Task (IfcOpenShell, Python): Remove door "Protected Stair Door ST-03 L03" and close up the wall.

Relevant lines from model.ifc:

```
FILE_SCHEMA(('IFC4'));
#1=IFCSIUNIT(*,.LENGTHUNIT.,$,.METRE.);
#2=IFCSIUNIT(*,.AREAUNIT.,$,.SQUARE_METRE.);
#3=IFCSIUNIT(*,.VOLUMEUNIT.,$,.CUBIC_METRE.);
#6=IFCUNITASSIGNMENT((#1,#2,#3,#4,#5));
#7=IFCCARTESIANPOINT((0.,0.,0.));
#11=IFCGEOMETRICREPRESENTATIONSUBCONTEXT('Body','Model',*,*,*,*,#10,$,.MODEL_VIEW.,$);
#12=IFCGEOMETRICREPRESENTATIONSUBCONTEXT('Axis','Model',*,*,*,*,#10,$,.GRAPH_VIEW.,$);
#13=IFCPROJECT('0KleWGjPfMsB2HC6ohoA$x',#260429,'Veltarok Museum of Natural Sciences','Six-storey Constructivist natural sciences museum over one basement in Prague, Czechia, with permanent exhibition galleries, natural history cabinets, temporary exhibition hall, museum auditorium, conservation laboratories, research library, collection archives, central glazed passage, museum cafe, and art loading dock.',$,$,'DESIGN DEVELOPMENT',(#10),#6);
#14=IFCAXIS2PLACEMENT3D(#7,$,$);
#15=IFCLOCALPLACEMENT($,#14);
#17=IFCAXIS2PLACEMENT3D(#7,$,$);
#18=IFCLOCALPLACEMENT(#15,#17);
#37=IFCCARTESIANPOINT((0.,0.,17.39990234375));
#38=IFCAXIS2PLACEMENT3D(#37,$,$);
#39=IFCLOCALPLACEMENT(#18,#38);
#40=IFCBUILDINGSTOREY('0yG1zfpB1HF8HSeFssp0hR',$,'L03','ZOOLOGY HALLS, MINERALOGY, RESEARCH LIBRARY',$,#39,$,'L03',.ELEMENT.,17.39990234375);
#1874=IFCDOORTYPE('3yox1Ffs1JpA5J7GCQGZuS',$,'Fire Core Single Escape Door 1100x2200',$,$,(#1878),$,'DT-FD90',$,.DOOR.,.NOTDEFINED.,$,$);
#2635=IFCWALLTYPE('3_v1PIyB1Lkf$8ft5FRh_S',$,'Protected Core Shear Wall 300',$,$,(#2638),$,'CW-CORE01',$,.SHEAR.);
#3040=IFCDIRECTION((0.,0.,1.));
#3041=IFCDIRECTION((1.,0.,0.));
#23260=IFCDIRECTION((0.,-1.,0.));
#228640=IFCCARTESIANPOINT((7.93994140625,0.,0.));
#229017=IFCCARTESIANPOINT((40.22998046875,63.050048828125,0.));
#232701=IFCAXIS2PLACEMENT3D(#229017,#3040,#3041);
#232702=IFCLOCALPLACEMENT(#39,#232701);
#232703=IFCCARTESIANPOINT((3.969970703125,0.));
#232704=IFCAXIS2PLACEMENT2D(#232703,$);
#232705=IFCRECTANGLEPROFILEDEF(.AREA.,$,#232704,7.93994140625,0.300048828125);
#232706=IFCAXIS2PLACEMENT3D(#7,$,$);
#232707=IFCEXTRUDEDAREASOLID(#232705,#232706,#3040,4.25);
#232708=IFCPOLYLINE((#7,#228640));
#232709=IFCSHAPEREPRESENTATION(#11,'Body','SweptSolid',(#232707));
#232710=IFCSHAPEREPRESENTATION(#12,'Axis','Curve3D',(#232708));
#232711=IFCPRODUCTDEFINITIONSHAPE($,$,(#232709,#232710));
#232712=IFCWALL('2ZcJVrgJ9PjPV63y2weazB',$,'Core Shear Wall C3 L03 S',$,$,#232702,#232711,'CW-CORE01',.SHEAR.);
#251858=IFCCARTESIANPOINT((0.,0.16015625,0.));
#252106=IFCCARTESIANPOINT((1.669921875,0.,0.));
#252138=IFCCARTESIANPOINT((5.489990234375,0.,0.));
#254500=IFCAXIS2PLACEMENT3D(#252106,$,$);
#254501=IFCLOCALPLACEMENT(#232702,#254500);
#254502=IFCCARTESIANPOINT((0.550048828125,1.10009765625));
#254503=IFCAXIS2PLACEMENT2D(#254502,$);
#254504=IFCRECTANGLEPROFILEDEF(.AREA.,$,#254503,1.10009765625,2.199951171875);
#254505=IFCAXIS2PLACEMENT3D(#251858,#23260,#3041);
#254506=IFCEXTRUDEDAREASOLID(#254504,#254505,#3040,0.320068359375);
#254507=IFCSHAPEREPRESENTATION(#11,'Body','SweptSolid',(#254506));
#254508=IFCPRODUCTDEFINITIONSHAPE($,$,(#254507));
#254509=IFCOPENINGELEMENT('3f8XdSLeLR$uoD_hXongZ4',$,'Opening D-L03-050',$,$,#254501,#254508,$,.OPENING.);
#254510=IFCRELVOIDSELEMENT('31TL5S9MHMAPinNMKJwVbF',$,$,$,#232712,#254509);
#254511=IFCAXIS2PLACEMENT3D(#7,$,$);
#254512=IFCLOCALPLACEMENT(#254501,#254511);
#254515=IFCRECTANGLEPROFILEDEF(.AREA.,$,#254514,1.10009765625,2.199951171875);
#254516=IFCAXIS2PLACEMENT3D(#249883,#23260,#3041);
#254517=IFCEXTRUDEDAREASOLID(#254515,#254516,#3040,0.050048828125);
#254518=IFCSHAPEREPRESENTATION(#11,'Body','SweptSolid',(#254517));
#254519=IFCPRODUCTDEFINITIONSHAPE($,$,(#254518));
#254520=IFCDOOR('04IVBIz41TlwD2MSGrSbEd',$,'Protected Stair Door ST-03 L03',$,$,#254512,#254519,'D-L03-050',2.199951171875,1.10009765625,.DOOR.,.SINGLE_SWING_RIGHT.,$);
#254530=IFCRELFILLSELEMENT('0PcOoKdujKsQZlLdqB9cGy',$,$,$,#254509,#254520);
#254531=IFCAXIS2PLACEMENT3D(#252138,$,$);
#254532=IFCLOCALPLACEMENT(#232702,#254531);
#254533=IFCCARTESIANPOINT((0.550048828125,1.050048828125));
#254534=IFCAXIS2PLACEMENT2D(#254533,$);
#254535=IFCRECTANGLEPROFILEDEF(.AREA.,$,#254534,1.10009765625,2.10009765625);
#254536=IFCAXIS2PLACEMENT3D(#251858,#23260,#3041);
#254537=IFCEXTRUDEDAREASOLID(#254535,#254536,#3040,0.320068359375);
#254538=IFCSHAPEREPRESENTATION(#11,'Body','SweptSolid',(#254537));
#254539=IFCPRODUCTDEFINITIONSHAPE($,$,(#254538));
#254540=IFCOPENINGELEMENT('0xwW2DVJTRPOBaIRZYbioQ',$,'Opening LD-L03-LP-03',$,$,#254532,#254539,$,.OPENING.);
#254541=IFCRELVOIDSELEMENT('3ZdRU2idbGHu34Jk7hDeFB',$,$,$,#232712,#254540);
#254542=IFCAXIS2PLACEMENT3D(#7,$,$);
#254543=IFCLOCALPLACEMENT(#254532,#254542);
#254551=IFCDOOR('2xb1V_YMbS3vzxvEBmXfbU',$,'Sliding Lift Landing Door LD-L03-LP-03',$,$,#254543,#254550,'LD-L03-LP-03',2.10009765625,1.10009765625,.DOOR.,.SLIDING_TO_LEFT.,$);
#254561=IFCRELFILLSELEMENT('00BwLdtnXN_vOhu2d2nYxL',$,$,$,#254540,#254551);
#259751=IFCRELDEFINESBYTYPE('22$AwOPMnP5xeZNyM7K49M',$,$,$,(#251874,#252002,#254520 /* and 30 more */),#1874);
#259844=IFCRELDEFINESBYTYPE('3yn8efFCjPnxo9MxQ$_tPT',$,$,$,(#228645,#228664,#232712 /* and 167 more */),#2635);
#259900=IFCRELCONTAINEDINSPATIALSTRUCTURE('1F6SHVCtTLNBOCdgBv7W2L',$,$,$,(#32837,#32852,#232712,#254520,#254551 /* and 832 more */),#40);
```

```python
import ifcopenshell
import ifcopenshell.api.feature
import ifcopenshell.api.root
import ifcopenshell.geom
import ifcopenshell.util.shape

model = ifcopenshell.open("model.ifc")
settings = ifcopenshell.geom.settings()


def volume(element):
    """Net volume in cubic metres, openings subtracted."""
    shape = ifcopenshell.geom.create_shape(settings, element)
    return ifcopenshell.util.shape.get_volume(shape.geometry)


door = model.by_guid("04IVBIz41TlwD2MSGrSbEd")
opening = door.FillsVoids[0].RelatingOpeningElement
wall = opening.VoidsElements[0].RelatingBuildingElement
before = volume(wall)

ifcopenshell.api.root.remove_product(model, product=door)
ifcopenshell.api.feature.remove_feature(model, feature=opening)

after = volume(wall)

print(f"wall volume {before:.3f} -> {after:.3f} m3")

model.write("model_rev.ifc")
```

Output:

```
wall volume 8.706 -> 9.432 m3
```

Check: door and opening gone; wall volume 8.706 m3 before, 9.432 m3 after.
